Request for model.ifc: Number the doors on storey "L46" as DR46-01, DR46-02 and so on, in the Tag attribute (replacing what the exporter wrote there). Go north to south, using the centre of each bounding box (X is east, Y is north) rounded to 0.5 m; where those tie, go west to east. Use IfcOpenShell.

First a look at what the model holds.

```python
import ifcopenshell
import ifcopenshell.util.element
import ifcopenshell.util.placement

model = ifcopenshell.open("model.ifc")
print(model.schema)
storey = next(s for s in model.by_type("IfcBuildingStorey") if s.Name == "L46")
doors = [e for e in ifcopenshell.util.element.get_decomposition(storey) if e.is_a("IfcDoor")]
for e in sorted(doors, key=lambda e: e.id()):
    origin = ifcopenshell.util.placement.get_local_placement(e.ObjectPlacement)[:3, 3]
    print(e.id(), e.Tag, e.Name, origin.round(2) + 0.0, sep=" | ")
```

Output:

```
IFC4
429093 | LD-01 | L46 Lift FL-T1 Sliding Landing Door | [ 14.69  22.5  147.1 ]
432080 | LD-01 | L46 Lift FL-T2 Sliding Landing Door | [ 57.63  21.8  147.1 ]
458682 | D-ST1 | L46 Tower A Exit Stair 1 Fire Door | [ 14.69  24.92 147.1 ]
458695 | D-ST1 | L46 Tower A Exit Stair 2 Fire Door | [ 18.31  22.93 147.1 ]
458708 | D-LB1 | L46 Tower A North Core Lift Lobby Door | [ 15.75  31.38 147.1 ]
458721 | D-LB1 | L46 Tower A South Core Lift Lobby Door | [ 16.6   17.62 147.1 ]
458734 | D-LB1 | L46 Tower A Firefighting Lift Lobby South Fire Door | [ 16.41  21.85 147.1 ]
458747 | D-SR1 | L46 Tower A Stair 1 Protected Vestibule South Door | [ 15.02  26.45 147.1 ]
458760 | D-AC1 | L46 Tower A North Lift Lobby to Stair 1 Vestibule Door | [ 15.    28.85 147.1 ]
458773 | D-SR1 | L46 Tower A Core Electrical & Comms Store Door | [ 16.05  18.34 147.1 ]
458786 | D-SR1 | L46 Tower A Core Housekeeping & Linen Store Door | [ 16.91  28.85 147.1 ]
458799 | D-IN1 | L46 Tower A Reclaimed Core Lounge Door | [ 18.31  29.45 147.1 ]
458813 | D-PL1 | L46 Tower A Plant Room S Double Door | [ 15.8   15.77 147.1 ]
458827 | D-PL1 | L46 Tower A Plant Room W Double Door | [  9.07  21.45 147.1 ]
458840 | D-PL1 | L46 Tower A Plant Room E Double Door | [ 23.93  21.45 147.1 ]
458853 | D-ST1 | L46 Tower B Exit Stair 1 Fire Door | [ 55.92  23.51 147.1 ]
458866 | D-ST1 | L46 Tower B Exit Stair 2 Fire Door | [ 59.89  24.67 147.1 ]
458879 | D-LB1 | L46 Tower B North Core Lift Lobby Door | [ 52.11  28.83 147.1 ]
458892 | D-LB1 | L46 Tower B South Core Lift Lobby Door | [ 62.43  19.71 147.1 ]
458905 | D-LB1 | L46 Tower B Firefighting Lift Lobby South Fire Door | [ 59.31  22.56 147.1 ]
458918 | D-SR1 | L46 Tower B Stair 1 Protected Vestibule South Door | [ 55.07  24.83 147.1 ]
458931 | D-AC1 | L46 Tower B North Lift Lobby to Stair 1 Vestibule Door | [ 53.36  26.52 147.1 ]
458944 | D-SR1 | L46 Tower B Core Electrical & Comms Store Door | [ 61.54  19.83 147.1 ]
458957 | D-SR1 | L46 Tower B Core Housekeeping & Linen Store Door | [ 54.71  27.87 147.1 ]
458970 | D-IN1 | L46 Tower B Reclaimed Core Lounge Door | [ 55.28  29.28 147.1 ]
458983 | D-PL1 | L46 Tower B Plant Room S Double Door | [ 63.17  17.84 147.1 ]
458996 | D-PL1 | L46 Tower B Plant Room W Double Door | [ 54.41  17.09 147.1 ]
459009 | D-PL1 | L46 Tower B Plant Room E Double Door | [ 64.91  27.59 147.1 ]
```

```python
import ifcopenshell
import ifcopenshell.geom
import ifcopenshell.util.element
import ifcopenshell.util.shape

model = ifcopenshell.open("model.ifc")
settings = ifcopenshell.geom.settings()
settings.set("use-world-coords", True)


def centre(element):
    shape = ifcopenshell.geom.create_shape(settings, element)
    return ifcopenshell.util.shape.get_bbox_centroid(shape.geometry)


storey = next(s for s in model.by_type("IfcBuildingStorey") if s.Name == "L46")
doors = [e for e in ifcopenshell.util.element.get_decomposition(storey) if e.is_a("IfcDoor")]

# Insertion points can sit at a corner or the storey origin, so sort by the geometry (in metres).
centres = {e: centre(e) for e in doors}
doors.sort(key=lambda e: (-round(centres[e][1] / 0.5), centres[e][0]))

for i, e in enumerate(doors, start=1):
    number = f"DR46-{i:02d}"
    e.Tag = number
    print(e.id(), number)

model.write("model_updated.ifc")
```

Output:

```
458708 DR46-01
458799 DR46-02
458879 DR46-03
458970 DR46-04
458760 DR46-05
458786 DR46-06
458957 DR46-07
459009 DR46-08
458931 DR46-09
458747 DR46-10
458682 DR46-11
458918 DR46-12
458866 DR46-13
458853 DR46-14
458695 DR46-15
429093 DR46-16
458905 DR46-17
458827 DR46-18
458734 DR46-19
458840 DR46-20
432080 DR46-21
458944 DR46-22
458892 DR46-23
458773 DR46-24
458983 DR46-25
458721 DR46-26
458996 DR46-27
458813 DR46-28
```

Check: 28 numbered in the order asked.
